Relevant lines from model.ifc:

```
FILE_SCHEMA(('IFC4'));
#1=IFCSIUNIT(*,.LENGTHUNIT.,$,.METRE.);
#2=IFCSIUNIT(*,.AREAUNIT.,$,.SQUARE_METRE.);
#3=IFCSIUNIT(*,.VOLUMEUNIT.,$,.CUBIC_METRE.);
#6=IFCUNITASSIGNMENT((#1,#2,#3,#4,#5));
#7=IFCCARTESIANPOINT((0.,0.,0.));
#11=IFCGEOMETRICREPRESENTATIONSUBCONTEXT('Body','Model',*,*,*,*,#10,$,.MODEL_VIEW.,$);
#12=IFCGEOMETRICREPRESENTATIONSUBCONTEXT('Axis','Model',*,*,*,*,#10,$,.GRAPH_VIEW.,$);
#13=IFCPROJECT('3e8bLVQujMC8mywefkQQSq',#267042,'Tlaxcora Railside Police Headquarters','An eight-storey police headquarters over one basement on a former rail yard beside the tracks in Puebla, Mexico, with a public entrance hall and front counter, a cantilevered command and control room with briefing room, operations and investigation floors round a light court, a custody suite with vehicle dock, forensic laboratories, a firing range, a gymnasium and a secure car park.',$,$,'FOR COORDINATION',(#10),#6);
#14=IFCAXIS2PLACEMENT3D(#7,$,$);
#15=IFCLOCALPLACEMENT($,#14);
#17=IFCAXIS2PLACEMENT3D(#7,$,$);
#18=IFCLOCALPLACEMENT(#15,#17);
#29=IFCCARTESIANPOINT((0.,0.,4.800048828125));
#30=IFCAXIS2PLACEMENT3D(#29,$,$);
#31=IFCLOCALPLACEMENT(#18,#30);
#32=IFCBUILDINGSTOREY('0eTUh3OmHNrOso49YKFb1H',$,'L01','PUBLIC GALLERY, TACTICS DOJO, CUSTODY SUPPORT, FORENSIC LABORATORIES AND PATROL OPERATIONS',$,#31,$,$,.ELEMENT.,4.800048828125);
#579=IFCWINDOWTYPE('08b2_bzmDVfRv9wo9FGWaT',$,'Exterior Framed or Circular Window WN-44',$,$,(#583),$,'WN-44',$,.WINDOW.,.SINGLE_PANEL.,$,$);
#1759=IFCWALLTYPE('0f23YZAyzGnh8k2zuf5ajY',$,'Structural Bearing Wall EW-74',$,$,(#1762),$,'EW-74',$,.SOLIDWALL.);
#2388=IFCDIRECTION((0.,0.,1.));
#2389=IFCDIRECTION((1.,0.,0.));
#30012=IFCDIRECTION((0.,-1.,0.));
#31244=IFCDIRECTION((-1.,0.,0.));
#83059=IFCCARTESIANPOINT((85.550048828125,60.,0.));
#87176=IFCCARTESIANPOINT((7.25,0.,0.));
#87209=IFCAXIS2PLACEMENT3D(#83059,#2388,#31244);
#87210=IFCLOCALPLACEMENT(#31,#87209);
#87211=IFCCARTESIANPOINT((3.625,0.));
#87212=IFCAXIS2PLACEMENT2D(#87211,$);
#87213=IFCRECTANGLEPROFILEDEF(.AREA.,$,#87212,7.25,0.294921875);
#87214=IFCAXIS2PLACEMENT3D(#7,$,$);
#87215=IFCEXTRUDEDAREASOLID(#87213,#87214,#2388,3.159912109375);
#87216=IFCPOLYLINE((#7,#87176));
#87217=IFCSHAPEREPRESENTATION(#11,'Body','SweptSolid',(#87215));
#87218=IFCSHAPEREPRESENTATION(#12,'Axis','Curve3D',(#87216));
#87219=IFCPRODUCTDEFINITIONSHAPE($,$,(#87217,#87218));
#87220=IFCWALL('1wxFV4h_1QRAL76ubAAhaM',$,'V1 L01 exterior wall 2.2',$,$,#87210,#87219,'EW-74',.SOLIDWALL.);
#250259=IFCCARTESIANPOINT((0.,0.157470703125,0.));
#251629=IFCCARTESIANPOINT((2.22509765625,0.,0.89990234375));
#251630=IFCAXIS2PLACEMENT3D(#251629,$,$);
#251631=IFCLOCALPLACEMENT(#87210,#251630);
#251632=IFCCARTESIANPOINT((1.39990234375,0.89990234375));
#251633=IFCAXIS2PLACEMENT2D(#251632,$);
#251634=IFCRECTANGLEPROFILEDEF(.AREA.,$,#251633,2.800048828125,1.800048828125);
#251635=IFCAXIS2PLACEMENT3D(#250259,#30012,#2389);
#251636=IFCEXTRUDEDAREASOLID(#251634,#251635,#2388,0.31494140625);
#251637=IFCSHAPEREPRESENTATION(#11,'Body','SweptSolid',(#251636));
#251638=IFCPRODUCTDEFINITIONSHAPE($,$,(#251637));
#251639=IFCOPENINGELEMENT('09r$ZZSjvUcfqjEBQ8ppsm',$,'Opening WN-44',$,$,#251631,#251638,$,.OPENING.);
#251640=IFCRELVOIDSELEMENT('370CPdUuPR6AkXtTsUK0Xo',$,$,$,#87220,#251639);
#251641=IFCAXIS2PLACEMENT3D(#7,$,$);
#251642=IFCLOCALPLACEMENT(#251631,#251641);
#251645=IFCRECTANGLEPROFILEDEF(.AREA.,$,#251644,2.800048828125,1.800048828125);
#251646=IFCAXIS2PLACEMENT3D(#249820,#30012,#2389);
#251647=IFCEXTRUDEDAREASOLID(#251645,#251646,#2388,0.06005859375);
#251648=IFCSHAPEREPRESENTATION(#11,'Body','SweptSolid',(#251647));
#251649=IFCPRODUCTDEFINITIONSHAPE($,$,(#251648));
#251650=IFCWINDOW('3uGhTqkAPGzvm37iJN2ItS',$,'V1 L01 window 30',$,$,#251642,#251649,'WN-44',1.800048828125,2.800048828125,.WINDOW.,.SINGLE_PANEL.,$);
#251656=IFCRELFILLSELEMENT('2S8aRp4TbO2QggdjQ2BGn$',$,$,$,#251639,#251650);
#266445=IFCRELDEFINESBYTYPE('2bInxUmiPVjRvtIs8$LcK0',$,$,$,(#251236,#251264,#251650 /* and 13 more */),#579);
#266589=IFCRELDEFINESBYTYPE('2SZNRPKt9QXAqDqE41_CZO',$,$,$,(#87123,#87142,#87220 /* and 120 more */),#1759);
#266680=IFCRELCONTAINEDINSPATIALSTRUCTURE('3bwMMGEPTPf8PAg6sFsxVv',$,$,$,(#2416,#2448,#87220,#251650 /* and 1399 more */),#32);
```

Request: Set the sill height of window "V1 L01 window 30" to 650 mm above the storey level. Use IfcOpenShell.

```python
import numpy as np
import ifcopenshell
import ifcopenshell.api.geometry
import ifcopenshell.geom
import ifcopenshell.util.element
import ifcopenshell.util.placement
import ifcopenshell.util.shape
import ifcopenshell.util.unit

model = ifcopenshell.open("model.ifc")
unit_scale = ifcopenshell.util.unit.calculate_unit_scale(model)

window = model.by_guid("3uGhTqkAPGzvm37iJN2ItS")
opening = window.FillsVoids[0].RelatingOpeningElement
storey = ifcopenshell.util.element.get_container(window, ifc_class="IfcBuildingStorey")
level = ifcopenshell.util.placement.get_local_placement(storey.ObjectPlacement)[2, 3]

# The opening's origin need not be at the sill, so measure its lowest point.
shape = ifcopenshell.geom.create_shape(ifcopenshell.geom.settings(), opening)
bottom = ifcopenshell.util.shape.get_shape_bottom_elevation(shape, shape.geometry) / unit_scale
dz = level + 0.65 / unit_scale - bottom

shift = np.array([0.0, 0.0, dz])
# The window is placed relative to its opening, so it follows when the opening moves.
matrix = ifcopenshell.util.placement.get_local_placement(opening.ObjectPlacement)
matrix[:3, 3] += shift
ifcopenshell.api.geometry.edit_object_placement(
    model, product=opening, matrix=matrix, is_si=False, should_transform_children=True
)

print(f"moved by {dz * unit_scale:+.3f} m")

model.write("model_edited.ifc")
```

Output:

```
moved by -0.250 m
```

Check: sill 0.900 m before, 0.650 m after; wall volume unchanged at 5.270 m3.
